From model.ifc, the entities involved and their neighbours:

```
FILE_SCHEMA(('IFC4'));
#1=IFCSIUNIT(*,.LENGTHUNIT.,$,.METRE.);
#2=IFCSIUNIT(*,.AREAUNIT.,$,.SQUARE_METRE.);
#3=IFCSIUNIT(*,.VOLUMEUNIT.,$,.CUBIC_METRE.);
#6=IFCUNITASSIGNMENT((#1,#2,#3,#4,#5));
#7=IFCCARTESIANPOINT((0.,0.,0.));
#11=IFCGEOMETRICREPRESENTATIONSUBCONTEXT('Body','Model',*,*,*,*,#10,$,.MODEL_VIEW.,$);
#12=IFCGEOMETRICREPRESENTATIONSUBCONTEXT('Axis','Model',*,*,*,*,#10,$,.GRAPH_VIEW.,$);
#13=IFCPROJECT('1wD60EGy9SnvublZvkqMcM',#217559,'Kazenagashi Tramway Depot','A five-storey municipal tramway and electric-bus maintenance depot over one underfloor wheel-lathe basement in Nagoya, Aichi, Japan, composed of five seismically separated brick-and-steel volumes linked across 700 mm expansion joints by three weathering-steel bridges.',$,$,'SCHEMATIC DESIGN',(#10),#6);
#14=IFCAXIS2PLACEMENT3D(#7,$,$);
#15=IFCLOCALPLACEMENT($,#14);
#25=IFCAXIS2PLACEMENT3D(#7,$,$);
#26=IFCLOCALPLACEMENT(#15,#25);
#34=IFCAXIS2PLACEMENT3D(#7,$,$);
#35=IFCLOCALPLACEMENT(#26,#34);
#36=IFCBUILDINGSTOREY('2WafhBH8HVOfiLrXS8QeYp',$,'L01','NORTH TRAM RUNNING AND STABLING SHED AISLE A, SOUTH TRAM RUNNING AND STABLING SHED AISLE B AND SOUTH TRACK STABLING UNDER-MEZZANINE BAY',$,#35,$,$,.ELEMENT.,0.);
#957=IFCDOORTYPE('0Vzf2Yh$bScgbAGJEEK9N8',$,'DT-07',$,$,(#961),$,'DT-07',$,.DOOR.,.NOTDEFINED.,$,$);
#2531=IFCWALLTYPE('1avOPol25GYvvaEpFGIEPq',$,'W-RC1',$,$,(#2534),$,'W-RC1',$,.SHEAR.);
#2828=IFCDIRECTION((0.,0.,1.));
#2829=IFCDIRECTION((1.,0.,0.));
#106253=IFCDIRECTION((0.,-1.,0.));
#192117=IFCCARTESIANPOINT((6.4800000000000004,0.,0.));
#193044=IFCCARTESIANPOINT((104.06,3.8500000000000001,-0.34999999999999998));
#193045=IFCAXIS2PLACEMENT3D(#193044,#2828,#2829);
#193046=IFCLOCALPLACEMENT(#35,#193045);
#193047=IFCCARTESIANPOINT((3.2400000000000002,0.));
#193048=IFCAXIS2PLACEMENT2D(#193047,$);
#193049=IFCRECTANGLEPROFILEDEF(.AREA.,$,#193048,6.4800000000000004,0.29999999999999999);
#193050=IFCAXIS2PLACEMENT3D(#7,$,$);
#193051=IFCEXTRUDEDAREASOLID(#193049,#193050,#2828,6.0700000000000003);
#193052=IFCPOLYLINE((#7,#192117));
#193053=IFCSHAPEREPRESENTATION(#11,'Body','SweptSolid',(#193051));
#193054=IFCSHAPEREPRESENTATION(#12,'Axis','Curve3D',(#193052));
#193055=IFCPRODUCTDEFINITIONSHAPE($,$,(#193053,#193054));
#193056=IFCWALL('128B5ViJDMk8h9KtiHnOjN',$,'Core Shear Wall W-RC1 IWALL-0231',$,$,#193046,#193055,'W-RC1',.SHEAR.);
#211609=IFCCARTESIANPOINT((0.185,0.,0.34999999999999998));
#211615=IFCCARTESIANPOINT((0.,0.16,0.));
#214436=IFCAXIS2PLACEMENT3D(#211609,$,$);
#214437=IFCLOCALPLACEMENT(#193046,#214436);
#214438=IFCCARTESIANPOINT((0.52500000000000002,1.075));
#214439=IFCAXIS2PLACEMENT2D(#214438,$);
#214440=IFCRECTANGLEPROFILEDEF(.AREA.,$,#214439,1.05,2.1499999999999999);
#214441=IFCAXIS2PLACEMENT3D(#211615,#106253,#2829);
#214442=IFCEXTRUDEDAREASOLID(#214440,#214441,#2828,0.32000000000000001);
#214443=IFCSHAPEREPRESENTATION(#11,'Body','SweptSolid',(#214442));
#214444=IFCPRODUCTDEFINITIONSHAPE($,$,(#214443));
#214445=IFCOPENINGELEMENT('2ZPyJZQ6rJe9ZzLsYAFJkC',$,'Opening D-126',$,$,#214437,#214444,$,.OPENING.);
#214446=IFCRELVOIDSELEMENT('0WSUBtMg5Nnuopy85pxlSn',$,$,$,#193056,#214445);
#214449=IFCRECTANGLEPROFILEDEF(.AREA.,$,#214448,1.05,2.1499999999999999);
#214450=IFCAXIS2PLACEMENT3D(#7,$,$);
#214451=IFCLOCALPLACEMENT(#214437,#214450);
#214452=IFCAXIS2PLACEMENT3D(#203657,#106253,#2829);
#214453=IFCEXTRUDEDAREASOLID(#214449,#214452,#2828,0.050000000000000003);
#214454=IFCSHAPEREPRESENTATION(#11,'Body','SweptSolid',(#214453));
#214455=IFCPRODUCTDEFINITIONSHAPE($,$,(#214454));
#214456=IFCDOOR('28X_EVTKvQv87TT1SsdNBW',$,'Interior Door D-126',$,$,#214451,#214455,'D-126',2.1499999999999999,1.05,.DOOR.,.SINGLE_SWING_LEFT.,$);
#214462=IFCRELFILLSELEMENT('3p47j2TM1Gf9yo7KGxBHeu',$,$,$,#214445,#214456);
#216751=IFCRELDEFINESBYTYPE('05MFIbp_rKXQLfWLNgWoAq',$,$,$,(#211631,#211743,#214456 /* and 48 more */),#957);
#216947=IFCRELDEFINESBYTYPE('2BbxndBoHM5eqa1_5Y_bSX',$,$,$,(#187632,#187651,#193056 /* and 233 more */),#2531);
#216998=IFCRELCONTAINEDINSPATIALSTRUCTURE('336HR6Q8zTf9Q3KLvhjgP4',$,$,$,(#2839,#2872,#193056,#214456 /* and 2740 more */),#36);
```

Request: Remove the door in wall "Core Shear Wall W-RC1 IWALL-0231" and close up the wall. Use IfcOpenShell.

```python
import ifcopenshell
import ifcopenshell.api.feature
import ifcopenshell.api.root
import ifcopenshell.geom
import ifcopenshell.util.shape

model = ifcopenshell.open("model.ifc")
settings = ifcopenshell.geom.settings()


def volume(element):
    """Net volume in cubic metres, openings subtracted."""
    shape = ifcopenshell.geom.create_shape(settings, element)
    return ifcopenshell.util.shape.get_volume(shape.geometry)


door = model.by_id(214456)
opening = door.FillsVoids[0].RelatingOpeningElement
wall = opening.VoidsElements[0].RelatingBuildingElement
before = volume(wall)

ifcopenshell.api.root.remove_product(model, product=door)
ifcopenshell.api.feature.remove_feature(model, feature=opening)

after = volume(wall)

print(f"wall volume {before:.3f} -> {after:.3f} m3")

model.write("model_rev.ifc")
```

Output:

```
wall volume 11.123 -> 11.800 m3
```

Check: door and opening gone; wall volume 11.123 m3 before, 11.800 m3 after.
